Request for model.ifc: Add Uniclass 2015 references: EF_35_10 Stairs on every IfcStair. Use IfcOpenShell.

First a look at what the model holds.

```python
import ifcopenshell

model = ifcopenshell.open("model.ifc")
print(model.schema)
print("classifications:", [c.Name for c in model.by_type("IfcClassification")])
for ifc_class in ("IfcDoor", "IfcRoof", "IfcStair", "IfcWall", "IfcWindow"):
    print(ifc_class, len(model.by_type(ifc_class)))
```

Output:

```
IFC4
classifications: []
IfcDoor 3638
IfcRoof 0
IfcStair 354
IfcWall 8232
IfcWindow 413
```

```python
import ifcopenshell
import ifcopenshell.api.classification

model = ifcopenshell.open("model.ifc")

system = ifcopenshell.api.classification.add_classification(model, classification="Uniclass 2015")

codes = {
    "IfcStair": ("EF_35_10", "Stairs"),
}
for ifc_class, (code, name) in codes.items():
    products = model.by_type(ifc_class)
    ifcopenshell.api.classification.add_reference(
        model, products=products, classification=system, identification=code, name=name
    )
    print(code, len(products))

model.write("model-out.ifc")
```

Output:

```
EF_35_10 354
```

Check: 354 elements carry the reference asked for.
